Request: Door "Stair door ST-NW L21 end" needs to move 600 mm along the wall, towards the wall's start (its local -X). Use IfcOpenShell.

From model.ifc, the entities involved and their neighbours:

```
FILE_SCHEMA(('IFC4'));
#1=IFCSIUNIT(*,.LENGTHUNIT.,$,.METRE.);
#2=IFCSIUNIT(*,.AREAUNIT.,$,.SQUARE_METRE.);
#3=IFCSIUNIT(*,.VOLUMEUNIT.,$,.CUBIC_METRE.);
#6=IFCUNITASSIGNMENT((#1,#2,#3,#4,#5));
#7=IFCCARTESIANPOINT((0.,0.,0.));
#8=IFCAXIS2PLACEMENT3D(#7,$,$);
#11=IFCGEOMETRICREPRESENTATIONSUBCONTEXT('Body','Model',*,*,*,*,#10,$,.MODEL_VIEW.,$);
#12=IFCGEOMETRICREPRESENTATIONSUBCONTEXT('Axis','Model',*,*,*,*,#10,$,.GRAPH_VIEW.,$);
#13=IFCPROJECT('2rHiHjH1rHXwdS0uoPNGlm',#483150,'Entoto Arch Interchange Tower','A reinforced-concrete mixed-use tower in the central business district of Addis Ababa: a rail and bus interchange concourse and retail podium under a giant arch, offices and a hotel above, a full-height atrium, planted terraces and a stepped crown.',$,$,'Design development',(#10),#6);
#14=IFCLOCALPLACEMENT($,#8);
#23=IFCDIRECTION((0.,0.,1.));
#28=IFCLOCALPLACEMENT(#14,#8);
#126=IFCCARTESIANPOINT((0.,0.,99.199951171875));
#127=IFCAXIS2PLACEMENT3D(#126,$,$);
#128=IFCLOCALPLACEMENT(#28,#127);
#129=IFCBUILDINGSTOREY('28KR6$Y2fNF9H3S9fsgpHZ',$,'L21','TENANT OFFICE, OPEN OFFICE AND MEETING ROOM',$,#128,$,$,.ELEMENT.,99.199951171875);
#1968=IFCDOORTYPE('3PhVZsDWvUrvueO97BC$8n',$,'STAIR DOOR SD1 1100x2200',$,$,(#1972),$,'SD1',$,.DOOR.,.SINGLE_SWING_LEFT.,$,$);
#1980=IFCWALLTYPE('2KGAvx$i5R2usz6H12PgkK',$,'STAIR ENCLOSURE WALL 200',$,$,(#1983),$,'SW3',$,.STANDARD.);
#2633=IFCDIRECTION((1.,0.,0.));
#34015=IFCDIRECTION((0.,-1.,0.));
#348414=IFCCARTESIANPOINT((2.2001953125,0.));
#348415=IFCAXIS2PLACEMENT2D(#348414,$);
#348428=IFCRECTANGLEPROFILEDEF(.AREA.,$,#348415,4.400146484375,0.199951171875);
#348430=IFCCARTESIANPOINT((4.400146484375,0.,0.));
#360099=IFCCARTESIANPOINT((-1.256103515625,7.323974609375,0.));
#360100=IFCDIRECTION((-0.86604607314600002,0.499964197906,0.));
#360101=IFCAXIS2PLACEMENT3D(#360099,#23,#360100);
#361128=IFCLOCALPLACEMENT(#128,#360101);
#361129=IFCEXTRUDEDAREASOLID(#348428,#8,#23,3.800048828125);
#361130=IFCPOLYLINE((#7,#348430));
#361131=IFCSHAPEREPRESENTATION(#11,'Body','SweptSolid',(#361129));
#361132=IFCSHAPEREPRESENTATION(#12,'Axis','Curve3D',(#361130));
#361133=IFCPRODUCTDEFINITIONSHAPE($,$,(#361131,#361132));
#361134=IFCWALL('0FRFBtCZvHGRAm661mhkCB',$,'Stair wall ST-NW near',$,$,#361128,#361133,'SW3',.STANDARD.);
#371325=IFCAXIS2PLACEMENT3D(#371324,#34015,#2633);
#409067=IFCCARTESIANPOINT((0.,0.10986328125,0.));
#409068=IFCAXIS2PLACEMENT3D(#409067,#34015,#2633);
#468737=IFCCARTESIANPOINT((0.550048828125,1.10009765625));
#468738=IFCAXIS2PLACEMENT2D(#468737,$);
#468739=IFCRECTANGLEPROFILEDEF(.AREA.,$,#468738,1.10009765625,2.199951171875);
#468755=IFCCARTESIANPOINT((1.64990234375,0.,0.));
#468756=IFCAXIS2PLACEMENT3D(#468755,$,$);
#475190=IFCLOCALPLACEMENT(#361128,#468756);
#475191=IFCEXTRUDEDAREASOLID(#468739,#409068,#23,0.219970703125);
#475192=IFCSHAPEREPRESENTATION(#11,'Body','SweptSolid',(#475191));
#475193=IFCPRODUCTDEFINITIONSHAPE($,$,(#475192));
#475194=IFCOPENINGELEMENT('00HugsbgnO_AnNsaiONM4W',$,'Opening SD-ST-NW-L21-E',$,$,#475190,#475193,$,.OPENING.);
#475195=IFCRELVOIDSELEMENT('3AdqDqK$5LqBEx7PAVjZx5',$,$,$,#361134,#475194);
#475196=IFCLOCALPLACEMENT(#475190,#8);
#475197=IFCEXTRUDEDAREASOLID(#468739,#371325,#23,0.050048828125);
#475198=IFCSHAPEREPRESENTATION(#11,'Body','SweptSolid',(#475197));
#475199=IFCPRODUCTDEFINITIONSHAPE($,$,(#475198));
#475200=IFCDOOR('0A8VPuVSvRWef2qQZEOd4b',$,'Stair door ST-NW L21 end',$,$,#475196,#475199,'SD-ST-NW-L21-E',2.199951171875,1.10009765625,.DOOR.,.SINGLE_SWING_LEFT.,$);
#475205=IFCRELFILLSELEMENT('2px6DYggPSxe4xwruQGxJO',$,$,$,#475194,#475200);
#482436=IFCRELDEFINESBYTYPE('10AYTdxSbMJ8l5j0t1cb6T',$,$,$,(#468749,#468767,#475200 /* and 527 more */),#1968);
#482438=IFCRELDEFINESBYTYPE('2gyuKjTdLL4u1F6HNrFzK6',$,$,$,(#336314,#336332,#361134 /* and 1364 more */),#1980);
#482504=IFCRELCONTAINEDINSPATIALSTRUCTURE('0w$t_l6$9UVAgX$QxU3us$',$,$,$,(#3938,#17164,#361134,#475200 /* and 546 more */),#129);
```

```python
import ifcopenshell
import ifcopenshell.api.geometry
import ifcopenshell.util.placement

model = ifcopenshell.open("model.ifc")

door = model.by_id(475200)
opening = door.FillsVoids[0].RelatingOpeningElement
wall = opening.VoidsElements[0].RelatingBuildingElement

wall_matrix = ifcopenshell.util.placement.get_local_placement(wall.ObjectPlacement)
shift = wall_matrix[:3, 0] * -0.6
before = ifcopenshell.util.placement.get_local_placement(door.ObjectPlacement)[:3, 3].copy()

# The door is placed relative to its opening, so it follows when the opening moves.
matrix = ifcopenshell.util.placement.get_local_placement(opening.ObjectPlacement)
matrix[:3, 3] += shift
ifcopenshell.api.geometry.edit_object_placement(
    model, product=opening, matrix=matrix, is_si=False, should_transform_children=True
)

after = ifcopenshell.util.placement.get_local_placement(door.ObjectPlacement)[:3, 3]
print("door moved by", (after - before).round(3) + 0.0)

model.write("model_rev.ifc")
```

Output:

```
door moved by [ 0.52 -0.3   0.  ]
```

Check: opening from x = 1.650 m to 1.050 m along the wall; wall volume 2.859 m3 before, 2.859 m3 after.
